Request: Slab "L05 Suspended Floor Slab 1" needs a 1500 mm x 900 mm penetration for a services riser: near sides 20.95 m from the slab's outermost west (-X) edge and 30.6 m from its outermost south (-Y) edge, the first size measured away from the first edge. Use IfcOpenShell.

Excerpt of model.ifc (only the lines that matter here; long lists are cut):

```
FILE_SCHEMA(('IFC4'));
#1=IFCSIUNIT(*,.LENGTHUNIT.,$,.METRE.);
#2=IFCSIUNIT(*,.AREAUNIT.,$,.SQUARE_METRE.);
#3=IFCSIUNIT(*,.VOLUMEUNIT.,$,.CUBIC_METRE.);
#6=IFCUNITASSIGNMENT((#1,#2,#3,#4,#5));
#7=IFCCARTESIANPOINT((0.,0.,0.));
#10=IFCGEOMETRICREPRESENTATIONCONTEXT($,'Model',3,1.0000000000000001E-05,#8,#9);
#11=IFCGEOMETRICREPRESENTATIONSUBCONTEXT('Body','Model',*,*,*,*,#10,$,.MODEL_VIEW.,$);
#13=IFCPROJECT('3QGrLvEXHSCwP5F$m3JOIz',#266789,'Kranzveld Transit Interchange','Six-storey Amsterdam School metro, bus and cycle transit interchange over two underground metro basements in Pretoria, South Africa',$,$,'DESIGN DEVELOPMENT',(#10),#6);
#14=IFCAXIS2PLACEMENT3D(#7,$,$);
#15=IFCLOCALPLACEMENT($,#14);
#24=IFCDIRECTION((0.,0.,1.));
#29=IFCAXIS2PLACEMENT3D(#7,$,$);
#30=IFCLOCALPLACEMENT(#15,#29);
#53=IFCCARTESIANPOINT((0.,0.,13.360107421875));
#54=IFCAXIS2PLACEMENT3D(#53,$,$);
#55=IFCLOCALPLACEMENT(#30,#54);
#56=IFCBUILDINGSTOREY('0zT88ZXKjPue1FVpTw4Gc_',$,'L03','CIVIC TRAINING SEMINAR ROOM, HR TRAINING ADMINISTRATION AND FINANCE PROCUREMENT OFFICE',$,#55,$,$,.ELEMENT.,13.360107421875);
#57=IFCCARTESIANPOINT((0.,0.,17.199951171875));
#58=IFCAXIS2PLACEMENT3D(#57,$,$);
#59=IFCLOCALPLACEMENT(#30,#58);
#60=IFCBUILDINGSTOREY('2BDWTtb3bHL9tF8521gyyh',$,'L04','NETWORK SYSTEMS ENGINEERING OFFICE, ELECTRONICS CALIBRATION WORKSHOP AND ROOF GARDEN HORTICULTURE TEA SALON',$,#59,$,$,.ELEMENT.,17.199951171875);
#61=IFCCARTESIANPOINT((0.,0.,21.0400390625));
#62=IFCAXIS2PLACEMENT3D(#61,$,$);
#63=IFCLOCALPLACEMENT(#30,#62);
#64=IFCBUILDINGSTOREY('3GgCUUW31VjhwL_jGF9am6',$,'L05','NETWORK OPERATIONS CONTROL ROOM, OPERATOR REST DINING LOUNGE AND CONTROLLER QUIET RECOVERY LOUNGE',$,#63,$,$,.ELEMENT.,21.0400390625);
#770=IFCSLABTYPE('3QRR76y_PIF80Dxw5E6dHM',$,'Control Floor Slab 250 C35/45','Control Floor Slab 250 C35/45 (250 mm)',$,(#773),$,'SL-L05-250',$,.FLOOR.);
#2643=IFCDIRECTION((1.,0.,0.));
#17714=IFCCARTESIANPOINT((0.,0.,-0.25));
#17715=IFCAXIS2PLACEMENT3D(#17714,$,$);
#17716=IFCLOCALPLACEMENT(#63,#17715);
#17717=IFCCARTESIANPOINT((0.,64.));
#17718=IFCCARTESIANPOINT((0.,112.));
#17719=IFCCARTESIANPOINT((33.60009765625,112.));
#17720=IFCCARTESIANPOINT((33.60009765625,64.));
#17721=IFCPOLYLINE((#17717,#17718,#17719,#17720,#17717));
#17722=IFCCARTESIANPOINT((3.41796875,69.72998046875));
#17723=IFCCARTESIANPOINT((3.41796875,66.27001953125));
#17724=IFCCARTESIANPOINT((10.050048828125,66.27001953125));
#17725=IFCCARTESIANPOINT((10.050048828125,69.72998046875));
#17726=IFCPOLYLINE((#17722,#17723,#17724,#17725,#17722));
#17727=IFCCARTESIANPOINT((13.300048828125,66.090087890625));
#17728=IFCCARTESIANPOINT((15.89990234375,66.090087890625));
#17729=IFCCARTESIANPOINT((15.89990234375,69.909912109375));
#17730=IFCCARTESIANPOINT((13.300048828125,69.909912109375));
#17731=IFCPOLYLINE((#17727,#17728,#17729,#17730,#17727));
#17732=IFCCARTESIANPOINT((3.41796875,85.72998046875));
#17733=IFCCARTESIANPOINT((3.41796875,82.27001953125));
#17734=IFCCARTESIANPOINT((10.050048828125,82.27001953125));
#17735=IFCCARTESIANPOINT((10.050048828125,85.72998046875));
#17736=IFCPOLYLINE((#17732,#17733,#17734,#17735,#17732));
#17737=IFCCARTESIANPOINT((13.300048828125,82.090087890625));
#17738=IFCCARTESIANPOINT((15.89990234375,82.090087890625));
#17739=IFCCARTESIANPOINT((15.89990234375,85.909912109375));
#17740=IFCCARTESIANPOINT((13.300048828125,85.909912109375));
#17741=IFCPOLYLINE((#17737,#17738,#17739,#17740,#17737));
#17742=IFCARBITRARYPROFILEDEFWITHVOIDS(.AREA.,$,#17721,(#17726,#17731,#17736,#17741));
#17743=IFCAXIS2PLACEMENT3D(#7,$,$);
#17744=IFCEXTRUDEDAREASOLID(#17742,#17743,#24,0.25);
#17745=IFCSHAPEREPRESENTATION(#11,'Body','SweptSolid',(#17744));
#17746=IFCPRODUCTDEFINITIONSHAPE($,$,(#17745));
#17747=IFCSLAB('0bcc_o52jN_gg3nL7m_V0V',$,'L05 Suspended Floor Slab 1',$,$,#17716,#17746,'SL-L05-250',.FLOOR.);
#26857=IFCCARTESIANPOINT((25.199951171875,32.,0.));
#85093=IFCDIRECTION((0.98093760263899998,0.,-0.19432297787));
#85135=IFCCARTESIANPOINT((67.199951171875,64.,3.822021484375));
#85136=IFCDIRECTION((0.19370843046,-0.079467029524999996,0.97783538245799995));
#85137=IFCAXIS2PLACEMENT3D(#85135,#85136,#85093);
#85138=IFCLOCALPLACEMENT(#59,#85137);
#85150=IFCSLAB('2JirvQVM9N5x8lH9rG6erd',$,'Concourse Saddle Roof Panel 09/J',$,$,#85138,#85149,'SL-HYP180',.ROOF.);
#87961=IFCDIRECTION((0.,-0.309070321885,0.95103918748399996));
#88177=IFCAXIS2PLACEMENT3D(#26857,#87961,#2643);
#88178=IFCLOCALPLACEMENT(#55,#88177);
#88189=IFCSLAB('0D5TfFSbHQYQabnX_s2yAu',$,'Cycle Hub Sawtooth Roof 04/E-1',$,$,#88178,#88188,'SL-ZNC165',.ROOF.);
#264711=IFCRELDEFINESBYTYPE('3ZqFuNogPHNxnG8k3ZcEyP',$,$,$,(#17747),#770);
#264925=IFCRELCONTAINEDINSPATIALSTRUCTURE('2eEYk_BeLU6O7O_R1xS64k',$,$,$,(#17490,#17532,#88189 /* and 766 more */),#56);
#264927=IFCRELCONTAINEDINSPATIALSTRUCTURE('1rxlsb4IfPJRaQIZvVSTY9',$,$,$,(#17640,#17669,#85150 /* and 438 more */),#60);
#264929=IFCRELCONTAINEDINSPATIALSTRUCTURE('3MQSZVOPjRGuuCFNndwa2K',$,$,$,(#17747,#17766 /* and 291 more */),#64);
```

```python
import numpy as np
import ifcopenshell
import ifcopenshell.api.feature
import ifcopenshell.api.geometry
import ifcopenshell.api.root
import ifcopenshell.geom
import ifcopenshell.util.placement
import ifcopenshell.util.representation
import ifcopenshell.util.shape
import ifcopenshell.util.unit

model = ifcopenshell.open("model.ifc")
unit_scale = ifcopenshell.util.unit.calculate_unit_scale(model)
settings = ifcopenshell.geom.settings()


def volume(element):
    """Net volume in cubic metres, openings subtracted."""
    shape = ifcopenshell.geom.create_shape(settings, element)
    return ifcopenshell.util.shape.get_volume(shape.geometry)


slab = model.by_id(17747)
before = volume(slab)

# Extent in the slab's own axes, in metres. The edges named are its -X and -Y sides.
slab_shape = ifcopenshell.geom.create_shape(settings, slab)
vertices = ifcopenshell.util.shape.get_vertices(slab_shape.geometry)
x_min, y_min, bottom = vertices.min(axis=0)
top = vertices[:, 2].max()

opening = ifcopenshell.api.root.create_entity(model, ifc_class="IfcOpeningElement", name="Services riser opening", predefined_type="OPENING")
context = ifcopenshell.util.representation.get_context(model, "Model", "Body", "MODEL_VIEW")
width, depth = 1.5, 0.9
outline = [(0.0, 0.0), (width, 0.0), (width, depth), (0.0, depth), (0.0, 0.0)]
# Overshoot both faces by 50 mm so the cut is clean.
shape = ifcopenshell.api.geometry.add_slab_representation(
    model, context=context, depth=top - bottom + 0.1, polyline=outline
)
ifcopenshell.api.geometry.assign_representation(model, product=opening, representation=shape)

matrix = ifcopenshell.util.placement.get_local_placement(slab.ObjectPlacement)
matrix[:, 3] = matrix @ np.append(np.array([x_min + 20.95, y_min + 30.6, bottom - 0.05]) / unit_scale, 1.0)
ifcopenshell.api.geometry.edit_object_placement(model, product=opening, matrix=matrix, is_si=False)
ifcopenshell.api.feature.add_feature(model, feature=opening, element=slab)

after = volume(slab)

print(f"slab volume {before:.3f} -> {after:.3f} m3")

model.write("model_updated.ifc")
```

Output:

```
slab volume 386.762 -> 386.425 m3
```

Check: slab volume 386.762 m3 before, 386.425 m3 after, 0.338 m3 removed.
